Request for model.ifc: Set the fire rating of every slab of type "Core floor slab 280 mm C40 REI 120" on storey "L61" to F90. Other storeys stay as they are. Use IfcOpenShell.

First a look at what the model holds.

```python
import ifcopenshell
import ifcopenshell.util.element

model = ifcopenshell.open("model.ifc")
print(model.schema)
storey = next(s for s in model.by_type("IfcBuildingStorey") if s.Name == "L61")
slabs = [e for e in ifcopenshell.util.element.get_decomposition(storey) if e.is_a("IfcSlab")]
seen = {}
for e in slabs:
    element_type = ifcopenshell.util.element.get_type(e)
    key = (element_type.Name if element_type != e and element_type else None, ifcopenshell.util.element.get_pset(e, "Pset_SlabCommon", "FireRating"))
    seen[key] = seen.get(key, 0) + 1
for (name, value), count in sorted(seen.items(), key=str):
    print(count, "x", name, "|", value)
```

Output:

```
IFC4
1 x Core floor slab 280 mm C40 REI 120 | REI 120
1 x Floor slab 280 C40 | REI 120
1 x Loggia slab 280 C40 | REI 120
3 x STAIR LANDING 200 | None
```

```python
import ifcopenshell
import ifcopenshell.api.pset
import ifcopenshell.util.element

model = ifcopenshell.open("model.ifc")

storey = next(s for s in model.by_type("IfcBuildingStorey") if s.Name == "L61")
slabs = [e for e in ifcopenshell.util.element.get_decomposition(storey) if e.is_a("IfcSlab")]

count = 0
for e in slabs:
    element_type = ifcopenshell.util.element.get_type(e)
    if element_type in (None, e) or element_type.Name != "Core floor slab 280 mm C40 REI 120":
        continue
    # add_pset returns the element's existing set when there is one.
    pset = ifcopenshell.api.pset.add_pset(model, product=e, name="Pset_SlabCommon")
    ifcopenshell.api.pset.edit_pset(model, pset=pset, properties={"FireRating": "F90"})
    count += 1

print(count, "slabs updated")

model.write("model-out.ifc")
```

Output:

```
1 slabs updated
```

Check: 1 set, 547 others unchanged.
